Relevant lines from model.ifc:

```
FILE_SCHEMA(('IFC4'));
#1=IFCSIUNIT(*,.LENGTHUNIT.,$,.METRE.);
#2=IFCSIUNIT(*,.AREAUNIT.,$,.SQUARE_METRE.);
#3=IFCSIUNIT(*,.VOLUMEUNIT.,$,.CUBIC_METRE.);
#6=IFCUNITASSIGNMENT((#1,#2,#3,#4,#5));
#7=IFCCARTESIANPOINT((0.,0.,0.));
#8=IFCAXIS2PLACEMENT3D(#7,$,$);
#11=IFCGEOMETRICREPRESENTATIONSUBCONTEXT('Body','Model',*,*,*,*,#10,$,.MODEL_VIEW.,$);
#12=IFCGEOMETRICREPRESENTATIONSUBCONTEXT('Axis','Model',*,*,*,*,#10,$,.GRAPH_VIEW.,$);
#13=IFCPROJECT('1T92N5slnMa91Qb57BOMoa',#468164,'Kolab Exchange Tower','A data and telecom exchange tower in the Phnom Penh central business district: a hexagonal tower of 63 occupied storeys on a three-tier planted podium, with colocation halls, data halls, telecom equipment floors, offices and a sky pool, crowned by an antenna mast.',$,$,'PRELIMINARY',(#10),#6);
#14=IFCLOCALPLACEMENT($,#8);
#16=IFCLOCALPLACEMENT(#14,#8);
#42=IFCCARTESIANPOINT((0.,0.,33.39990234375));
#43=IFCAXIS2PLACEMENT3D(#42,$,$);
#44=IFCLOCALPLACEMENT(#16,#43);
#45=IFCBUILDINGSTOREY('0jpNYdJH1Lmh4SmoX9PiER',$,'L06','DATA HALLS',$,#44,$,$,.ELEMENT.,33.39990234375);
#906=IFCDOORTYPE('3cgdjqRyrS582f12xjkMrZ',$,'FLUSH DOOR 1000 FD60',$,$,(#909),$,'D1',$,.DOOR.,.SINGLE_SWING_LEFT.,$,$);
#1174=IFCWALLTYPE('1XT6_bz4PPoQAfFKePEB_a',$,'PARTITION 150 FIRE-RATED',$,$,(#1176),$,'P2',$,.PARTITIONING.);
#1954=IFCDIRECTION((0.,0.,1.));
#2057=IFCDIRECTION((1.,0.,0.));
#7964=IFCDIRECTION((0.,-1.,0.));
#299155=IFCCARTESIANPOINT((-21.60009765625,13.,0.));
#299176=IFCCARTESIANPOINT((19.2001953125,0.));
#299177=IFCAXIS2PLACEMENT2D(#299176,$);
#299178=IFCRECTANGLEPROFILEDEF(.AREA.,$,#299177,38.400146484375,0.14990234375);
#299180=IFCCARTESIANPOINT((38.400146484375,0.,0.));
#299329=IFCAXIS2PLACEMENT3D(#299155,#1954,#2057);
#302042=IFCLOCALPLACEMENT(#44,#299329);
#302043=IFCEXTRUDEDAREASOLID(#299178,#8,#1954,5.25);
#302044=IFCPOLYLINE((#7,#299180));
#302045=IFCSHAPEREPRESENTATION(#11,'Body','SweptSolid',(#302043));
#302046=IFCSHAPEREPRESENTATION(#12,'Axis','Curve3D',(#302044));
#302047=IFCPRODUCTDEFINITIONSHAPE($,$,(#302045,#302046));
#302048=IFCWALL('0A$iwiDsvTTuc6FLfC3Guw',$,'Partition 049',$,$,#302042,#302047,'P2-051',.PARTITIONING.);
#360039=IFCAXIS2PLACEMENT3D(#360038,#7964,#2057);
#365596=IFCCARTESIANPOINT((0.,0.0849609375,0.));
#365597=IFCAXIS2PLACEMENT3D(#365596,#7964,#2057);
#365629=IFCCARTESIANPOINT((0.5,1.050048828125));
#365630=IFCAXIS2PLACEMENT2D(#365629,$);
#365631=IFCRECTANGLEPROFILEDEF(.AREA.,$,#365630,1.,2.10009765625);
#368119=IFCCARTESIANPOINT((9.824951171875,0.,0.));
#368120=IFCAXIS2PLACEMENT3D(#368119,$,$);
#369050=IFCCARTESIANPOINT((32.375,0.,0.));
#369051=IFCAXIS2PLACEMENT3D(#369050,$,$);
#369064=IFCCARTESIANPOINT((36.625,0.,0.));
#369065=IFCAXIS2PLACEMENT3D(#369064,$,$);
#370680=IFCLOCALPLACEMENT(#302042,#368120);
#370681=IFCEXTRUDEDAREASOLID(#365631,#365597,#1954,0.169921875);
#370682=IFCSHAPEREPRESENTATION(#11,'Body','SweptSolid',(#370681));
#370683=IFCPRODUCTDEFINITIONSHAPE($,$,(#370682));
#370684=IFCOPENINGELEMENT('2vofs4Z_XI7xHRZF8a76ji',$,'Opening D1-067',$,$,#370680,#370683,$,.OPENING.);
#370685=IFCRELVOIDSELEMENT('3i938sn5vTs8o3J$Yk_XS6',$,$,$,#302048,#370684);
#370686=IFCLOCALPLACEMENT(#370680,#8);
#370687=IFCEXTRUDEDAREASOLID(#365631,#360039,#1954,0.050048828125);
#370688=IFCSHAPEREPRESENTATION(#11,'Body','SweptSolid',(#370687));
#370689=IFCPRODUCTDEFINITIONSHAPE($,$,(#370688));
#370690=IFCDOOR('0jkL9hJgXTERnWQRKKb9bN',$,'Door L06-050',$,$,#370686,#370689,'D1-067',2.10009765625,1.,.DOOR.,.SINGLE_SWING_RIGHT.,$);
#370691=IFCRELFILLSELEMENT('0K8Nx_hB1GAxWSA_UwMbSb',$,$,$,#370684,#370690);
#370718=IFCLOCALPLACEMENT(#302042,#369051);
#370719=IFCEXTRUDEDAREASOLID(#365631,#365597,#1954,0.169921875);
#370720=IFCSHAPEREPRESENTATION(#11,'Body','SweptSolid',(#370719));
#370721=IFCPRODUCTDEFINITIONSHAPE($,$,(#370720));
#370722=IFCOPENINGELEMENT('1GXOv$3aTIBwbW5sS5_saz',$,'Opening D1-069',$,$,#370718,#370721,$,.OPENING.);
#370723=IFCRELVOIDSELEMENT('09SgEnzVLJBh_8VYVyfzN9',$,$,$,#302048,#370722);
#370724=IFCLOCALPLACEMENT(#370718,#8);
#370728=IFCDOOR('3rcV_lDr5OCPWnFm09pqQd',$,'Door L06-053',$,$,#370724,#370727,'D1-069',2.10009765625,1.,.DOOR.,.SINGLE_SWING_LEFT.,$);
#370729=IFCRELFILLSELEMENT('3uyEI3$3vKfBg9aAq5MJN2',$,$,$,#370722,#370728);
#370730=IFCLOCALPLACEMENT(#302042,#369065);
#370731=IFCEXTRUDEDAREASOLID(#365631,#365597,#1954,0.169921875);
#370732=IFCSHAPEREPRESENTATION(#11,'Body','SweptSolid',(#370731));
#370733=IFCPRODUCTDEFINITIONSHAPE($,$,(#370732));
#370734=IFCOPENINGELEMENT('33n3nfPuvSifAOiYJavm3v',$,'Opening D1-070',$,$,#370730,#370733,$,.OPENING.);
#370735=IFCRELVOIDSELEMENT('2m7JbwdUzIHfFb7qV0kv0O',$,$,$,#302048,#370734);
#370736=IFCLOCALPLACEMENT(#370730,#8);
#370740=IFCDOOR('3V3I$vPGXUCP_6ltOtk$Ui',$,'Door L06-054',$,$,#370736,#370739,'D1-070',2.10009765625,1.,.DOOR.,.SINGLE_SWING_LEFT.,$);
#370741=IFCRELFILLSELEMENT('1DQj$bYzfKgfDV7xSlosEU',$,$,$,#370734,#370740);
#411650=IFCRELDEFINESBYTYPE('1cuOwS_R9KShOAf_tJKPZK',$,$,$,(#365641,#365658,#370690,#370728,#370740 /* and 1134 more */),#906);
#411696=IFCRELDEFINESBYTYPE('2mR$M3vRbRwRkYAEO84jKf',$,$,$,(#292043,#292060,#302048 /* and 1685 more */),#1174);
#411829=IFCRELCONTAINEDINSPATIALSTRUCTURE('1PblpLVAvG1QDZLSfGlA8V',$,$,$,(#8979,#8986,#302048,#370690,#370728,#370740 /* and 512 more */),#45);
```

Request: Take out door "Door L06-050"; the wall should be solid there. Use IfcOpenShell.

```python
import ifcopenshell
import ifcopenshell.api.feature
import ifcopenshell.api.root
import ifcopenshell.geom
import ifcopenshell.util.shape

model = ifcopenshell.open("model.ifc")
settings = ifcopenshell.geom.settings()


def volume(element):
    """Net volume in cubic metres, openings subtracted."""
    shape = ifcopenshell.geom.create_shape(settings, element)
    return ifcopenshell.util.shape.get_volume(shape.geometry)


door = model.by_guid("0jkL9hJgXTERnWQRKKb9bN")
opening = door.FillsVoids[0].RelatingOpeningElement
wall = opening.VoidsElements[0].RelatingBuildingElement
before = volume(wall)

ifcopenshell.api.root.remove_product(model, product=door)
ifcopenshell.api.feature.remove_feature(model, feature=opening)

after = volume(wall)

print(f"wall volume {before:.3f} -> {after:.3f} m3")

model.write("model_edited.ifc")
```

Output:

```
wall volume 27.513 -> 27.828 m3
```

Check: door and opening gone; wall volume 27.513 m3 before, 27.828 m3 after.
